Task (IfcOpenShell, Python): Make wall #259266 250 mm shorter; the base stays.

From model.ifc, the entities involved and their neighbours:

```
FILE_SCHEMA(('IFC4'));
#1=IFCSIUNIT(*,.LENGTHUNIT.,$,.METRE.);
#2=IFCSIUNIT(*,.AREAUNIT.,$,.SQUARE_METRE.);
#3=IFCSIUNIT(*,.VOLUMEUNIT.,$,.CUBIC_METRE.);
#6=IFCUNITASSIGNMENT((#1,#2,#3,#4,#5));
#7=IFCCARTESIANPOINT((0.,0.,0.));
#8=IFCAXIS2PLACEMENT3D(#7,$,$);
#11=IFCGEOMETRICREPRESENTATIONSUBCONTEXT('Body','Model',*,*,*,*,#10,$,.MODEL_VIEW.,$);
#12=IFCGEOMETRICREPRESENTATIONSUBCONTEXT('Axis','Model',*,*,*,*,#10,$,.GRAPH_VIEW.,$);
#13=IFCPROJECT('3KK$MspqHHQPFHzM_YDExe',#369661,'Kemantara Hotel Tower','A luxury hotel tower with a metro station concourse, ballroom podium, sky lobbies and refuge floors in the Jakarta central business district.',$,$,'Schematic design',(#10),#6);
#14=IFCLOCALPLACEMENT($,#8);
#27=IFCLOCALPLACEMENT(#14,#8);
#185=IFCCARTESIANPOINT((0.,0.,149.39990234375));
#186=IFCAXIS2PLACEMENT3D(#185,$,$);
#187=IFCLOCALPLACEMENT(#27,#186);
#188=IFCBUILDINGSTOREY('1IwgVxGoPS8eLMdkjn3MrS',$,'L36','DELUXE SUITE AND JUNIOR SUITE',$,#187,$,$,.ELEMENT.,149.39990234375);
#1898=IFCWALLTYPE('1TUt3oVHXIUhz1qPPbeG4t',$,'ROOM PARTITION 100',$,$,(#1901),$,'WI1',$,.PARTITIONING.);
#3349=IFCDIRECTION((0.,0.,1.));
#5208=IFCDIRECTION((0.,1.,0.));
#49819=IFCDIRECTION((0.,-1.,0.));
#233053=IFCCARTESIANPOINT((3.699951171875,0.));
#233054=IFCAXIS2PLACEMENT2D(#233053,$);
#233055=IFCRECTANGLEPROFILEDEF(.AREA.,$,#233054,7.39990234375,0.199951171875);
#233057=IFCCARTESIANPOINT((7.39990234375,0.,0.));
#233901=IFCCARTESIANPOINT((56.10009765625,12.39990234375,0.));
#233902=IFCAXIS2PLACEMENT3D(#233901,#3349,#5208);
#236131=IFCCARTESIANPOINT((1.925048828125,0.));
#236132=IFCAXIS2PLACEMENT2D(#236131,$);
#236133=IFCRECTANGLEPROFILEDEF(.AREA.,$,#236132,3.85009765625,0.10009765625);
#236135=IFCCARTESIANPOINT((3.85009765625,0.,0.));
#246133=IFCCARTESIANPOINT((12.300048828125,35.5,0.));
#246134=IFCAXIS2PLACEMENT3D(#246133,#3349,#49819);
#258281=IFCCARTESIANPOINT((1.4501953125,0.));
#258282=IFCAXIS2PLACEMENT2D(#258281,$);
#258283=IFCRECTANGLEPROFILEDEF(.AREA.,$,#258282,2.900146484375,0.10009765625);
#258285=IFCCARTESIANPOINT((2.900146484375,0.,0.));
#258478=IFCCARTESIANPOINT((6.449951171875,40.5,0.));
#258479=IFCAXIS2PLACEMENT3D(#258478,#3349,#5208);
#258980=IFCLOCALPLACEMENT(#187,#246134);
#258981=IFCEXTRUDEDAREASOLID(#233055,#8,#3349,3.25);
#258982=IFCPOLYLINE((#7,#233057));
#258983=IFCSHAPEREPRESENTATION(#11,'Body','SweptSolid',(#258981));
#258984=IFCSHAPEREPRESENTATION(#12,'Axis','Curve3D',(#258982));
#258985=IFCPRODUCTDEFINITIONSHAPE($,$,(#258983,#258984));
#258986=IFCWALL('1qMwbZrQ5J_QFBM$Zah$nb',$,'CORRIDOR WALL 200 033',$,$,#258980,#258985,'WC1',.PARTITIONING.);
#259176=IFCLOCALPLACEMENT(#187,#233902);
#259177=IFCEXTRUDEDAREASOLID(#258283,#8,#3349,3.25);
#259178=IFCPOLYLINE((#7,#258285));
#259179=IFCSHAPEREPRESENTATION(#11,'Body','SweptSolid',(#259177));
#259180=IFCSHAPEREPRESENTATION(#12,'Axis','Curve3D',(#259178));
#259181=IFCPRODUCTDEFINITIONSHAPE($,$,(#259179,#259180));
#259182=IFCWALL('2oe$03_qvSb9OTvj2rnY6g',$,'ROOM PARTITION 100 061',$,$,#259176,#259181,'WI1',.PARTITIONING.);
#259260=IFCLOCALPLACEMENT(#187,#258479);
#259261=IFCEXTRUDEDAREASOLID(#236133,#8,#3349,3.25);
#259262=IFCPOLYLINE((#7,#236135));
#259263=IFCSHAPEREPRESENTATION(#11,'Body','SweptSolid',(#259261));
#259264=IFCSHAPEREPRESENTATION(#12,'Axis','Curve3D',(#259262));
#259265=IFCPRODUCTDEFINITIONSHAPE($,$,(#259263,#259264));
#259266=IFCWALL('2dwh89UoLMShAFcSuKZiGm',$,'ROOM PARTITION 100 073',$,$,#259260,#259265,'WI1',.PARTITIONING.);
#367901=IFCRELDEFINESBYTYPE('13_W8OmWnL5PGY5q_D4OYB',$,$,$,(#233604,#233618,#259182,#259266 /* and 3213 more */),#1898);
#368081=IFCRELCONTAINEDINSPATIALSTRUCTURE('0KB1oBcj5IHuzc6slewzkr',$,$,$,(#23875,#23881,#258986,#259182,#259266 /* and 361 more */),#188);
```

```python
import ifcopenshell
import ifcopenshell.geom
import ifcopenshell.util.representation
import ifcopenshell.util.shape

model = ifcopenshell.open("model.ifc")
settings = ifcopenshell.geom.settings()


def volume(element):
    """Net volume in cubic metres, openings subtracted."""
    shape = ifcopenshell.geom.create_shape(settings, element)
    return ifcopenshell.util.shape.get_volume(shape.geometry)


wall = model.by_guid("2dwh89UoLMShAFcSuKZiGm")
before = volume(wall)

body = ifcopenshell.util.representation.get_representation(wall, "Model", "Body")
solid = body.Items[0]
old_height = solid.Depth
solid.Depth -= 0.25
after = volume(wall)

print(f"height {old_height:g} -> {solid.Depth:g}, volume {before:.3f} -> {after:.3f} m3")

model.write("model_updated.ifc")
```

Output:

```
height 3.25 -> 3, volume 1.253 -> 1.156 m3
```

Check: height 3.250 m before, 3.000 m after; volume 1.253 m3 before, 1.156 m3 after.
